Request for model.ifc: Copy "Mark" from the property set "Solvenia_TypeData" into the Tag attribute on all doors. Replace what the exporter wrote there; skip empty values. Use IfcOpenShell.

First a look at what the model holds.

```python
import ifcopenshell
import ifcopenshell.util.element

model = ifcopenshell.open("model.ifc")
print(model.schema)
doors = model.by_type("IfcDoor")
print(len(doors), "doors")
for e in doors[:8]:
    source = ifcopenshell.util.element.get_pset(e, "Solvenia_TypeData", "Mark")
    target = e.Tag
    print(e.id(), repr(source), repr(target), sep=" | ")
```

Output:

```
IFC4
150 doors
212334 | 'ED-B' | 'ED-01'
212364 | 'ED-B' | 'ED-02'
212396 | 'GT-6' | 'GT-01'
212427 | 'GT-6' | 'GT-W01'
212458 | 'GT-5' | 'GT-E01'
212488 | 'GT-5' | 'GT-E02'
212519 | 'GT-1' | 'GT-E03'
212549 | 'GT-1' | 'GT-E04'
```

```python
import ifcopenshell
import ifcopenshell.util.element

model = ifcopenshell.open("model.ifc")

count = 0
for e in model.by_type("IfcDoor"):
    value = ifcopenshell.util.element.get_pset(e, "Solvenia_TypeData", "Mark")
    current = e.Tag
    if not value or not value.strip() or current == value:
        continue
    e.Tag = value
    count += 1

print(count, "doors updated")

model.write("model_edited.ifc")
```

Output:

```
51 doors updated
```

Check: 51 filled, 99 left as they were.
